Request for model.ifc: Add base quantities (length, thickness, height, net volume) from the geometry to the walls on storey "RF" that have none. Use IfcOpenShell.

First a look at what the model holds.

```python
import ifcopenshell
import ifcopenshell.util.element
import ifcopenshell.util.unit

model = ifcopenshell.open("model.ifc")
print(model.schema)
for unit_type in ("LENGTHUNIT", "AREAUNIT", "VOLUMEUNIT"):
    print(unit_type, ifcopenshell.util.unit.calculate_unit_scale(model, unit_type))
storey = next(s for s in model.by_type("IfcBuildingStorey") if s.Name == "RF")
walls = [e for e in ifcopenshell.util.element.get_decomposition(storey) if e.is_a("IfcWall")]
for e in sorted(walls, key=lambda e: e.id()):
    print(e.id(), e.is_a(), e.Name, list(ifcopenshell.util.element.get_psets(e, qtos_only=True)), sep=" | ")
```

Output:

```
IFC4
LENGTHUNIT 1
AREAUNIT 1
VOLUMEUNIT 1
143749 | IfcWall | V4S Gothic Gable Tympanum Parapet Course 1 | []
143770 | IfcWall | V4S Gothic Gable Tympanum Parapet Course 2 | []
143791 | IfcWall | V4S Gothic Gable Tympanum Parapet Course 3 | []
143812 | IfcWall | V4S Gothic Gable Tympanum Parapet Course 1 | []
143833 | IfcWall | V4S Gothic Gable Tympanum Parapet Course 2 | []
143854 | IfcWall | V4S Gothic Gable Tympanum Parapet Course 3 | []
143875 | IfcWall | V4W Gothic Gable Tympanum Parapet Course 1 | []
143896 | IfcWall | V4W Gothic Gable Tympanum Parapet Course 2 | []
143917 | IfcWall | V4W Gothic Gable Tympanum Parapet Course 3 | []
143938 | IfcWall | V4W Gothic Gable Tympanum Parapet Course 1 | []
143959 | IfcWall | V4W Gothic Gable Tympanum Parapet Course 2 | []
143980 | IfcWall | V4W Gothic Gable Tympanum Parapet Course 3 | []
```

```python
import ifcopenshell
import ifcopenshell.api.pset
import ifcopenshell.geom
import ifcopenshell.util.element
import ifcopenshell.util.shape
import ifcopenshell.util.unit

model = ifcopenshell.open("model.ifc")
unit_scale = ifcopenshell.util.unit.calculate_unit_scale(model)
volume_scale = ifcopenshell.util.unit.calculate_unit_scale(model, "VOLUMEUNIT")
settings = ifcopenshell.geom.settings()

storey = next(s for s in model.by_type("IfcBuildingStorey") if s.Name == "RF")
walls = [e for e in ifcopenshell.util.element.get_decomposition(storey) if e.is_a("IfcWall")]

for e in sorted(walls, key=lambda e: e.id()):
    if ifcopenshell.util.element.get_psets(e, qtos_only=True, should_inherit=False):
        continue
    # Geometry comes back in metres, in the element's own axes.
    shape = ifcopenshell.geom.create_shape(settings, e)
    values = {
        "Length": ifcopenshell.util.shape.get_x(shape.geometry) / unit_scale,
        "Width": ifcopenshell.util.shape.get_y(shape.geometry) / unit_scale,
        "Height": ifcopenshell.util.shape.get_z(shape.geometry) / unit_scale,
        "NetVolume": ifcopenshell.util.shape.get_volume(shape.geometry) / volume_scale,
    }
    qto = ifcopenshell.api.pset.add_qto(model, product=e, name="Qto_WallBaseQuantities")
    ifcopenshell.api.pset.edit_qto(model, qto=qto, properties=values)
    print(e.id(), {k: round(v, 3) for k, v in values.items()})

model.write("model-out.ifc")
```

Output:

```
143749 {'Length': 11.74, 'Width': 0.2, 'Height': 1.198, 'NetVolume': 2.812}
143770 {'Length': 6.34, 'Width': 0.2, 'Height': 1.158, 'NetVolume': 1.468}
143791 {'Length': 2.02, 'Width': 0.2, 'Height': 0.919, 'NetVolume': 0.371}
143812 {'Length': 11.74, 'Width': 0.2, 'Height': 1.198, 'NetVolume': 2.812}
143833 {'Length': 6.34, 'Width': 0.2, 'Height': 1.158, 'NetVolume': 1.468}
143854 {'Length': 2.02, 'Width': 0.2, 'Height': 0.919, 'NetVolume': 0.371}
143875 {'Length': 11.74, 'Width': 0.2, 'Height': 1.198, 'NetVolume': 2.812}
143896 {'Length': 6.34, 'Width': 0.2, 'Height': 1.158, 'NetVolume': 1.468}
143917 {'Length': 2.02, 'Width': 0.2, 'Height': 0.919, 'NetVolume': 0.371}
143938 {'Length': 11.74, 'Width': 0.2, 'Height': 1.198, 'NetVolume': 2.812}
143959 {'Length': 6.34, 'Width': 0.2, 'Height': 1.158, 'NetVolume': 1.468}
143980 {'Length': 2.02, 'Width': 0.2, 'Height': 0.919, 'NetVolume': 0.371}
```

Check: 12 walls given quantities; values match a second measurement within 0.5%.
